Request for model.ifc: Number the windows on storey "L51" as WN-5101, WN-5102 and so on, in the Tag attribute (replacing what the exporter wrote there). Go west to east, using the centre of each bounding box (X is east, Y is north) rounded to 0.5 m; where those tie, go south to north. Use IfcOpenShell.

First a look at what the model holds.

```python
import ifcopenshell
import ifcopenshell.util.element
import ifcopenshell.util.placement

model = ifcopenshell.open("model.ifc")
print(model.schema)
storey = next(s for s in model.by_type("IfcBuildingStorey") if s.Name == "L51")
windows = [e for e in ifcopenshell.util.element.get_decomposition(storey) if e.is_a("IfcWindow")]
for e in sorted(windows, key=lambda e: e.id()):
    origin = ifcopenshell.util.placement.get_local_placement(e.ObjectPlacement)[:3, 3]
    print(e.id(), e.Tag, e.Name, origin.round(2) + 0.0, sep=" | ")
```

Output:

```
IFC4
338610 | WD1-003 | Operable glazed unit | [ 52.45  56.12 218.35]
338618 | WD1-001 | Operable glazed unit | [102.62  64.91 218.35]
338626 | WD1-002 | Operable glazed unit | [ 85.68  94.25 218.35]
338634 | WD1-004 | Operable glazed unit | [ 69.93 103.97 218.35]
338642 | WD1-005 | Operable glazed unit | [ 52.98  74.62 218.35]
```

```python
import ifcopenshell
import ifcopenshell.geom
import ifcopenshell.util.element
import ifcopenshell.util.shape

model = ifcopenshell.open("model.ifc")
settings = ifcopenshell.geom.settings()
settings.set("use-world-coords", True)


def centre(element):
    shape = ifcopenshell.geom.create_shape(settings, element)
    return ifcopenshell.util.shape.get_bbox_centroid(shape.geometry)


storey = next(s for s in model.by_type("IfcBuildingStorey") if s.Name == "L51")
windows = [e for e in ifcopenshell.util.element.get_decomposition(storey) if e.is_a("IfcWindow")]

# Insertion points can sit at a corner or the storey origin, so sort by the geometry (in metres).
centres = {e: centre(e) for e in windows}
windows.sort(key=lambda e: (round(centres[e][0] / 0.5), centres[e][1]))

for i, e in enumerate(windows, start=1):
    number = f"WN-51{i:02d}"
    e.Tag = number
    print(e.id(), number)

model.write("model_edited.ifc")
```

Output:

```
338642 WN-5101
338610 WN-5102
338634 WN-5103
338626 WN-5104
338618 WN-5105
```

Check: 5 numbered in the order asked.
